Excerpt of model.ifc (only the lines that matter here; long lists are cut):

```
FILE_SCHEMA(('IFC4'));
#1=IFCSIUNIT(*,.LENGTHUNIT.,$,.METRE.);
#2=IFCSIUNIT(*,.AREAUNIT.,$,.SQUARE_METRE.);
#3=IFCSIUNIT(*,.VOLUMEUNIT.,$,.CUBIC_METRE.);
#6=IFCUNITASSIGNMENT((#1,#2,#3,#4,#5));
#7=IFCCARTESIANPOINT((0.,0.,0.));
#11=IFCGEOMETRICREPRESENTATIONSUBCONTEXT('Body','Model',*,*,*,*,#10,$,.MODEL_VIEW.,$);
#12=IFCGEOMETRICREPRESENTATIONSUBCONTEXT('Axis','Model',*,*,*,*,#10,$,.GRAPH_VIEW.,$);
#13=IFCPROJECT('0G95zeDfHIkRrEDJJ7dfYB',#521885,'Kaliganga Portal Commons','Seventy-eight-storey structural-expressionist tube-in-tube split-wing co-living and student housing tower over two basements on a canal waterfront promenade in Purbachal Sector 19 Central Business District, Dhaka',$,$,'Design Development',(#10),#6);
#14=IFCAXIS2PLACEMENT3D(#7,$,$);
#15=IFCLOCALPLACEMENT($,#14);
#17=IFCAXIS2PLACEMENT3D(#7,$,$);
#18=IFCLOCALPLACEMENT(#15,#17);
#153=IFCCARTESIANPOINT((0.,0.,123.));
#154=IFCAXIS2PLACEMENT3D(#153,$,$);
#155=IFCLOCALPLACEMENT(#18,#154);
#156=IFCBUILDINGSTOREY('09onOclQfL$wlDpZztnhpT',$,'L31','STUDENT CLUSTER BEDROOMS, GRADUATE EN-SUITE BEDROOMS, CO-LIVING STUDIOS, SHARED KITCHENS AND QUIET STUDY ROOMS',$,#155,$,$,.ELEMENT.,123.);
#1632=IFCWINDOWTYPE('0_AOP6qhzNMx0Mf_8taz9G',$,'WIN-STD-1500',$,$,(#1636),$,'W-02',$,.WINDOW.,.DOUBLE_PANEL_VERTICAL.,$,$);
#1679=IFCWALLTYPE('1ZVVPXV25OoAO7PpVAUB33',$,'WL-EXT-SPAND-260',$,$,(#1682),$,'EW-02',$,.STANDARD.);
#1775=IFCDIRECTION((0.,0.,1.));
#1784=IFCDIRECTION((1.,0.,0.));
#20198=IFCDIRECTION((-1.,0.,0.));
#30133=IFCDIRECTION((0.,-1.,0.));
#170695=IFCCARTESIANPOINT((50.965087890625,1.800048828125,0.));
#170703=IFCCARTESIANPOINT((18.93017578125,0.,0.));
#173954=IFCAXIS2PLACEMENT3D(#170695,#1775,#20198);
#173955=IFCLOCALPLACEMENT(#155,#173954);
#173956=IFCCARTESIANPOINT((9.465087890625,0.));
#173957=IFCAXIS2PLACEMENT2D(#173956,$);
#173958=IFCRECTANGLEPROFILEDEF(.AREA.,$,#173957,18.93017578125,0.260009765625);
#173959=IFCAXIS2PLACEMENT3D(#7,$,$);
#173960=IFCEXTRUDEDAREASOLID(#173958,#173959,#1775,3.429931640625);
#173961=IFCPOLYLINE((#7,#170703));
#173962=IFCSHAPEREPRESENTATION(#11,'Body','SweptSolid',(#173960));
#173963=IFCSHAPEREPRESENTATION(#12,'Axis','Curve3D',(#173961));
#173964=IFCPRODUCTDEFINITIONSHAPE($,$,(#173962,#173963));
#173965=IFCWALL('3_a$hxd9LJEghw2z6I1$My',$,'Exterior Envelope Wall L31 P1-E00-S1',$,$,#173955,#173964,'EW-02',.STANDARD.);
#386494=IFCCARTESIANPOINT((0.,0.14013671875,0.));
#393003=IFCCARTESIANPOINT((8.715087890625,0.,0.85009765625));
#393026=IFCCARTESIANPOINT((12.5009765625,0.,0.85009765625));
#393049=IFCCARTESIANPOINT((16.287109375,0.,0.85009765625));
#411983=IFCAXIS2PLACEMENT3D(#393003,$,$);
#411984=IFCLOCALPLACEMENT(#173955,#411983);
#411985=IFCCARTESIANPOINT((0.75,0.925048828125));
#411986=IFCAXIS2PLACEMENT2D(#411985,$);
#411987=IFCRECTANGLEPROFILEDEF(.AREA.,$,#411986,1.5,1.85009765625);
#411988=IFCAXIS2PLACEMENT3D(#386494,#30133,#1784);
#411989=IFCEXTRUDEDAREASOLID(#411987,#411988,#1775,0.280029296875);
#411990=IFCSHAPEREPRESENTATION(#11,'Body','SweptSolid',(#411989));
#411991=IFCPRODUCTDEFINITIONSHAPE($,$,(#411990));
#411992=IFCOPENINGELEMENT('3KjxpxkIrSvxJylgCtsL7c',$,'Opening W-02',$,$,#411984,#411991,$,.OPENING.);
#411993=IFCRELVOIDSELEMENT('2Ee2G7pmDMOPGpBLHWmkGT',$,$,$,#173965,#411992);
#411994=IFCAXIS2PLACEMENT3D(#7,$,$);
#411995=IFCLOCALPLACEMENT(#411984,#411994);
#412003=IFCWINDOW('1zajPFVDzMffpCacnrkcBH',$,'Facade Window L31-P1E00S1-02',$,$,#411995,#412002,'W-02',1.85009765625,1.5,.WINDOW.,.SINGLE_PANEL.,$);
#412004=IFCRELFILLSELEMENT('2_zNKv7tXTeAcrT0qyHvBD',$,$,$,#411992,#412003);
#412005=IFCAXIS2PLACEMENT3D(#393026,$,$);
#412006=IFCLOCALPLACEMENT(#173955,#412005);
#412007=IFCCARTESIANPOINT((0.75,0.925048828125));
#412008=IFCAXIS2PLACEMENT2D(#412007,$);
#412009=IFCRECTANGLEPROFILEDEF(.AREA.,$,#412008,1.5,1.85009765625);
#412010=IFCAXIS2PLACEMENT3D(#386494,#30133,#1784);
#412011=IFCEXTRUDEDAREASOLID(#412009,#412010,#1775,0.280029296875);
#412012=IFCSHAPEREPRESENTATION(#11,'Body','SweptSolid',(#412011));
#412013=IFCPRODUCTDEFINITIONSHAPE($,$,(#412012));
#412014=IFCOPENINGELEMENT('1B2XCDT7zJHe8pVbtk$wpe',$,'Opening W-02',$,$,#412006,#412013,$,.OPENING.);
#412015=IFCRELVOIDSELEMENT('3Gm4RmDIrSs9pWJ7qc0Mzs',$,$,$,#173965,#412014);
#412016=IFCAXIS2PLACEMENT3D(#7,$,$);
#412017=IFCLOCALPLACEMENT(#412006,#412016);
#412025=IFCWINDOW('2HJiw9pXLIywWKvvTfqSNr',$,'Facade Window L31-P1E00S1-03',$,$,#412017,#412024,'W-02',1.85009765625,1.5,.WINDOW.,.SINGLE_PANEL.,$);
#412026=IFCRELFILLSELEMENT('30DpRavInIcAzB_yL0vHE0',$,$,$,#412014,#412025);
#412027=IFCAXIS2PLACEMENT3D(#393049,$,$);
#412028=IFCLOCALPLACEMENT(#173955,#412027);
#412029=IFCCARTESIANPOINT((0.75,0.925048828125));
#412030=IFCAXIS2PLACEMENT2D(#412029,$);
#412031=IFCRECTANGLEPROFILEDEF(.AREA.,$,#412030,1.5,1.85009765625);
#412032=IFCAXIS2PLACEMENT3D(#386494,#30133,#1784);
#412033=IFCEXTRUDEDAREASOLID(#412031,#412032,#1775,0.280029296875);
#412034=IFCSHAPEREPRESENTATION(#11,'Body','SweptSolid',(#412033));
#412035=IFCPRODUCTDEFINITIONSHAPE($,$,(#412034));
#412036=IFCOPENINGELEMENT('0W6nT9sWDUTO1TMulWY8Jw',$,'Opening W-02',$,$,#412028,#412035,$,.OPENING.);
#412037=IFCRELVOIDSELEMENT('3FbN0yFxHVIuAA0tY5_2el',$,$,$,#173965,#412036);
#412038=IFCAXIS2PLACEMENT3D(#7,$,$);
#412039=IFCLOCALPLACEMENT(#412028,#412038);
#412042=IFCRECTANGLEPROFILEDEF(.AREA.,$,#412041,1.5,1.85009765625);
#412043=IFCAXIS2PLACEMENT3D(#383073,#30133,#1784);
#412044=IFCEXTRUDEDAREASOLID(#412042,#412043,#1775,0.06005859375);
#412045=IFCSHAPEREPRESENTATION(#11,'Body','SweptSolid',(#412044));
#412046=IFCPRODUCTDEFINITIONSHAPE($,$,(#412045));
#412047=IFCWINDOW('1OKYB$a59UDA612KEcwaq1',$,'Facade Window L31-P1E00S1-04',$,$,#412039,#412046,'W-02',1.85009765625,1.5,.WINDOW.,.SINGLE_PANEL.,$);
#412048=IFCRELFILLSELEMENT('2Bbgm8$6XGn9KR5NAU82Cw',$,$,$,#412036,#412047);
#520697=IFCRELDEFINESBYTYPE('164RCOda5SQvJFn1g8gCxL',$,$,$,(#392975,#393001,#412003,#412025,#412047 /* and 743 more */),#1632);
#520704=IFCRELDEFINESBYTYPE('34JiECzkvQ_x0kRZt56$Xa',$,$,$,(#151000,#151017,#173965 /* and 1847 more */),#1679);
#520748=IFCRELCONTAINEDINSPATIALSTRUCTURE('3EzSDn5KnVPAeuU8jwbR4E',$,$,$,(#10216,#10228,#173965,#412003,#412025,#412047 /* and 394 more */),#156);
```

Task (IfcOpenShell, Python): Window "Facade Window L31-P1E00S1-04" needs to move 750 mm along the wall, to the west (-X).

```python
import ifcopenshell
import ifcopenshell.api.geometry
import ifcopenshell.util.placement
import ifcopenshell.util.unit

model = ifcopenshell.open("model.ifc")
unit_scale = ifcopenshell.util.unit.calculate_unit_scale(model)

window = model.by_guid("1OKYB$a59UDA612KEcwaq1")
opening = window.FillsVoids[0].RelatingOpeningElement
wall = opening.VoidsElements[0].RelatingBuildingElement

wall_matrix = ifcopenshell.util.placement.get_local_placement(wall.ObjectPlacement)
shift = wall_matrix[:3, 0] * 0.75 / unit_scale
before = ifcopenshell.util.placement.get_local_placement(window.ObjectPlacement)[:3, 3].copy()

# The window is placed relative to its opening, so it follows when the opening moves.
matrix = ifcopenshell.util.placement.get_local_placement(opening.ObjectPlacement)
matrix[:3, 3] += shift
ifcopenshell.api.geometry.edit_object_placement(
    model, product=opening, matrix=matrix, is_si=False, should_transform_children=True
)

after = ifcopenshell.util.placement.get_local_placement(window.ObjectPlacement)[:3, 3]
print("window moved by", (after - before).round(3) + 0.0)

model.write("model-out.ifc")
```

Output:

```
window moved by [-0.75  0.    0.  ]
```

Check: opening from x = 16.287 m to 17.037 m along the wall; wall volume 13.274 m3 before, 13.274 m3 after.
